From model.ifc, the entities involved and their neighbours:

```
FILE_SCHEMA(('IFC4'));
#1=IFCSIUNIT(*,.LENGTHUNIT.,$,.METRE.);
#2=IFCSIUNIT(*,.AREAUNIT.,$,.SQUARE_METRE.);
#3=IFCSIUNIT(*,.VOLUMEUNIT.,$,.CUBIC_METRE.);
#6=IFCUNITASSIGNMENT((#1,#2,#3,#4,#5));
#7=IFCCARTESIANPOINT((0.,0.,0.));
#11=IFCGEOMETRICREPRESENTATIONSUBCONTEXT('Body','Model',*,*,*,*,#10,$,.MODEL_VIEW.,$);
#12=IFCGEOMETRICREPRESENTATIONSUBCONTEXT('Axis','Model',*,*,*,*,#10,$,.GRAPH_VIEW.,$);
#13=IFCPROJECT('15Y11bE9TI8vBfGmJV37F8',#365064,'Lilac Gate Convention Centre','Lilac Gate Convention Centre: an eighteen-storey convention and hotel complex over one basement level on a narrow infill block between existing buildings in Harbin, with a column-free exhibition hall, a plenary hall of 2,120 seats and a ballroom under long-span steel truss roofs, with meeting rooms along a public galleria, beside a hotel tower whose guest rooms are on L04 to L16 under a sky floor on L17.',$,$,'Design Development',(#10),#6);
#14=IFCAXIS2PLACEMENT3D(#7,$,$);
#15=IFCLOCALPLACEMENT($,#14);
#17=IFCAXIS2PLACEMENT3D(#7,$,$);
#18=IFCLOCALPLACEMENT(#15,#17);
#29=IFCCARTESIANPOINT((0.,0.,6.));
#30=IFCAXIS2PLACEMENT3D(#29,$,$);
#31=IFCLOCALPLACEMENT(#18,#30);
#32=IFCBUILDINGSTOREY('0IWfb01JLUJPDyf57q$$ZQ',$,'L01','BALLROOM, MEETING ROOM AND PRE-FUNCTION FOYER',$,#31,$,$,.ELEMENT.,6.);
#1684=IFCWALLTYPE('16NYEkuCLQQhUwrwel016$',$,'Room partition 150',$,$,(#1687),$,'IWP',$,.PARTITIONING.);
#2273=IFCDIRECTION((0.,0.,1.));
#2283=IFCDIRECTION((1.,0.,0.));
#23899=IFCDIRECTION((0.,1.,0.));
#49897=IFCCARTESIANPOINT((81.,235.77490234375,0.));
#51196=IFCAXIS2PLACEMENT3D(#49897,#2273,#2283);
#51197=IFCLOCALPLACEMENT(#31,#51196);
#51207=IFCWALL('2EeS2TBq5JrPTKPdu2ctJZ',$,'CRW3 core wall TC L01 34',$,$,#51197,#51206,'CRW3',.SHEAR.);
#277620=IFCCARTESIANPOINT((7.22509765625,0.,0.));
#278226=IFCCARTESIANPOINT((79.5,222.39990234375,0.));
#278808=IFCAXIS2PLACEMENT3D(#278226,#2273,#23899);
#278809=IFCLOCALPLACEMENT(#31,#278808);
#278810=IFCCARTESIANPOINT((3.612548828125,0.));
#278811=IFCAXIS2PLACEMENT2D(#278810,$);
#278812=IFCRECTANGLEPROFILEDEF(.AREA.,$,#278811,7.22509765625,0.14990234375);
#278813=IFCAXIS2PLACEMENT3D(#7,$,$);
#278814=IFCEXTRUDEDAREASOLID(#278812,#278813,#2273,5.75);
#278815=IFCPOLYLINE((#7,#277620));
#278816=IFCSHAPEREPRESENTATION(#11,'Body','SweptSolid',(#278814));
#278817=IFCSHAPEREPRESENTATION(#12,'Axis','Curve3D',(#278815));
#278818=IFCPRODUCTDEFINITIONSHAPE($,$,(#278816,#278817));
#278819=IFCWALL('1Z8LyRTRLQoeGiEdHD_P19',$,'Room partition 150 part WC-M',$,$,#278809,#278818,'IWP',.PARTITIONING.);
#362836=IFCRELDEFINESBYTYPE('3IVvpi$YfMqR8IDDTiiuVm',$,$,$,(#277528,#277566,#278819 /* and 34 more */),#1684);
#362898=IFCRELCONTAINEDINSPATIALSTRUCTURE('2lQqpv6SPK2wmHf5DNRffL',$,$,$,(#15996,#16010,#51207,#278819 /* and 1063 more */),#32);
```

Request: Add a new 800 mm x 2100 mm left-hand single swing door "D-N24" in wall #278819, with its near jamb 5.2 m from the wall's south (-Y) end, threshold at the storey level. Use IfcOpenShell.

```python
import numpy as np
import ifcopenshell
import ifcopenshell.api.feature
import ifcopenshell.api.geometry
import ifcopenshell.api.root
import ifcopenshell.api.spatial
import ifcopenshell.geom
import ifcopenshell.util.element
import ifcopenshell.util.placement
import ifcopenshell.util.representation
import ifcopenshell.util.shape
import ifcopenshell.util.unit

model = ifcopenshell.open("model.ifc")
unit_scale = ifcopenshell.util.unit.calculate_unit_scale(model)
settings = ifcopenshell.geom.settings()


def volume(element):
    """Net volume in cubic metres, openings subtracted."""
    shape = ifcopenshell.geom.create_shape(settings, element)
    return ifcopenshell.util.shape.get_volume(shape.geometry)


wall = model.by_guid("1Z8LyRTRLQoeGiEdHD_P19")
storey = ifcopenshell.util.element.get_container(wall, ifc_class="IfcBuildingStorey")
context = ifcopenshell.util.representation.get_context(model, "Model", "Body", "MODEL_VIEW")
before = volume(wall)

width, height, from_end, sill = 0.8, 2.1, 5.2, 0.0  # metres

# The wall runs along its own X axis, and the end named is its -X end.
wall_shape = ifcopenshell.geom.create_shape(settings, wall)
x, y, z = ifcopenshell.util.shape.get_vertices(wall_shape.geometry).T
start = x.min() + from_end
face, thickness = float(y.min()), float(y.max() - y.min())
wall_matrix = ifcopenshell.util.placement.get_local_placement(wall.ObjectPlacement)
level = ifcopenshell.util.placement.get_local_placement(storey.ObjectPlacement)[2, 3]


def in_wall(x, y):
    """Placement at x, y metres in the wall's axes, at sill height."""
    matrix = wall_matrix.copy()
    matrix[:, 3] = wall_matrix @ np.array([x / unit_scale, y / unit_scale, 0.0, 1.0])
    matrix[2, 3] = level + sill / unit_scale
    return matrix


# Opening: a box that overshoots both wall faces by 50 mm.
opening = ifcopenshell.api.root.create_entity(model, ifc_class="IfcOpeningElement", predefined_type="OPENING")
box = ifcopenshell.api.geometry.add_wall_representation(
    model, context=context, length=width, height=height, thickness=thickness + 0.1
)
ifcopenshell.api.geometry.assign_representation(model, product=opening, representation=box)
ifcopenshell.api.geometry.edit_object_placement(model, product=opening, matrix=in_wall(start, face - 0.05), is_si=False)
ifcopenshell.api.feature.add_feature(model, feature=opening, element=wall)

door = ifcopenshell.api.root.create_entity(model, ifc_class="IfcDoor", name="D-N24", predefined_type="DOOR")
door.OverallWidth, door.OverallHeight = width / unit_scale, height / unit_scale
door.OperationType = "SINGLE_SWING_LEFT"
body = ifcopenshell.api.geometry.add_door_representation(
    model,
    context=context,
    overall_width=door.OverallWidth,
    overall_height=door.OverallHeight,
    operation_type="SINGLE_SWING_LEFT",
    lining_properties={"LiningDepth": thickness / unit_scale, "ThresholdDepth": thickness / unit_scale},
)
ifcopenshell.api.geometry.assign_representation(model, product=door, representation=body)
ifcopenshell.api.spatial.assign_container(model, products=[door], relating_structure=storey)
ifcopenshell.api.feature.add_filling(model, opening=opening, element=door)

# The lining spans the wall, so the door starts at the wall face.
ifcopenshell.api.geometry.edit_object_placement(model, product=door, matrix=in_wall(start, face), is_si=False)

after = volume(wall)

print(f"wall volume {before:.3f} -> {after:.3f} m3")

model.write("model_edited.ifc")
```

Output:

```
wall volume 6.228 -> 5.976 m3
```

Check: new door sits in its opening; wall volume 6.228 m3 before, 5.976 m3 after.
